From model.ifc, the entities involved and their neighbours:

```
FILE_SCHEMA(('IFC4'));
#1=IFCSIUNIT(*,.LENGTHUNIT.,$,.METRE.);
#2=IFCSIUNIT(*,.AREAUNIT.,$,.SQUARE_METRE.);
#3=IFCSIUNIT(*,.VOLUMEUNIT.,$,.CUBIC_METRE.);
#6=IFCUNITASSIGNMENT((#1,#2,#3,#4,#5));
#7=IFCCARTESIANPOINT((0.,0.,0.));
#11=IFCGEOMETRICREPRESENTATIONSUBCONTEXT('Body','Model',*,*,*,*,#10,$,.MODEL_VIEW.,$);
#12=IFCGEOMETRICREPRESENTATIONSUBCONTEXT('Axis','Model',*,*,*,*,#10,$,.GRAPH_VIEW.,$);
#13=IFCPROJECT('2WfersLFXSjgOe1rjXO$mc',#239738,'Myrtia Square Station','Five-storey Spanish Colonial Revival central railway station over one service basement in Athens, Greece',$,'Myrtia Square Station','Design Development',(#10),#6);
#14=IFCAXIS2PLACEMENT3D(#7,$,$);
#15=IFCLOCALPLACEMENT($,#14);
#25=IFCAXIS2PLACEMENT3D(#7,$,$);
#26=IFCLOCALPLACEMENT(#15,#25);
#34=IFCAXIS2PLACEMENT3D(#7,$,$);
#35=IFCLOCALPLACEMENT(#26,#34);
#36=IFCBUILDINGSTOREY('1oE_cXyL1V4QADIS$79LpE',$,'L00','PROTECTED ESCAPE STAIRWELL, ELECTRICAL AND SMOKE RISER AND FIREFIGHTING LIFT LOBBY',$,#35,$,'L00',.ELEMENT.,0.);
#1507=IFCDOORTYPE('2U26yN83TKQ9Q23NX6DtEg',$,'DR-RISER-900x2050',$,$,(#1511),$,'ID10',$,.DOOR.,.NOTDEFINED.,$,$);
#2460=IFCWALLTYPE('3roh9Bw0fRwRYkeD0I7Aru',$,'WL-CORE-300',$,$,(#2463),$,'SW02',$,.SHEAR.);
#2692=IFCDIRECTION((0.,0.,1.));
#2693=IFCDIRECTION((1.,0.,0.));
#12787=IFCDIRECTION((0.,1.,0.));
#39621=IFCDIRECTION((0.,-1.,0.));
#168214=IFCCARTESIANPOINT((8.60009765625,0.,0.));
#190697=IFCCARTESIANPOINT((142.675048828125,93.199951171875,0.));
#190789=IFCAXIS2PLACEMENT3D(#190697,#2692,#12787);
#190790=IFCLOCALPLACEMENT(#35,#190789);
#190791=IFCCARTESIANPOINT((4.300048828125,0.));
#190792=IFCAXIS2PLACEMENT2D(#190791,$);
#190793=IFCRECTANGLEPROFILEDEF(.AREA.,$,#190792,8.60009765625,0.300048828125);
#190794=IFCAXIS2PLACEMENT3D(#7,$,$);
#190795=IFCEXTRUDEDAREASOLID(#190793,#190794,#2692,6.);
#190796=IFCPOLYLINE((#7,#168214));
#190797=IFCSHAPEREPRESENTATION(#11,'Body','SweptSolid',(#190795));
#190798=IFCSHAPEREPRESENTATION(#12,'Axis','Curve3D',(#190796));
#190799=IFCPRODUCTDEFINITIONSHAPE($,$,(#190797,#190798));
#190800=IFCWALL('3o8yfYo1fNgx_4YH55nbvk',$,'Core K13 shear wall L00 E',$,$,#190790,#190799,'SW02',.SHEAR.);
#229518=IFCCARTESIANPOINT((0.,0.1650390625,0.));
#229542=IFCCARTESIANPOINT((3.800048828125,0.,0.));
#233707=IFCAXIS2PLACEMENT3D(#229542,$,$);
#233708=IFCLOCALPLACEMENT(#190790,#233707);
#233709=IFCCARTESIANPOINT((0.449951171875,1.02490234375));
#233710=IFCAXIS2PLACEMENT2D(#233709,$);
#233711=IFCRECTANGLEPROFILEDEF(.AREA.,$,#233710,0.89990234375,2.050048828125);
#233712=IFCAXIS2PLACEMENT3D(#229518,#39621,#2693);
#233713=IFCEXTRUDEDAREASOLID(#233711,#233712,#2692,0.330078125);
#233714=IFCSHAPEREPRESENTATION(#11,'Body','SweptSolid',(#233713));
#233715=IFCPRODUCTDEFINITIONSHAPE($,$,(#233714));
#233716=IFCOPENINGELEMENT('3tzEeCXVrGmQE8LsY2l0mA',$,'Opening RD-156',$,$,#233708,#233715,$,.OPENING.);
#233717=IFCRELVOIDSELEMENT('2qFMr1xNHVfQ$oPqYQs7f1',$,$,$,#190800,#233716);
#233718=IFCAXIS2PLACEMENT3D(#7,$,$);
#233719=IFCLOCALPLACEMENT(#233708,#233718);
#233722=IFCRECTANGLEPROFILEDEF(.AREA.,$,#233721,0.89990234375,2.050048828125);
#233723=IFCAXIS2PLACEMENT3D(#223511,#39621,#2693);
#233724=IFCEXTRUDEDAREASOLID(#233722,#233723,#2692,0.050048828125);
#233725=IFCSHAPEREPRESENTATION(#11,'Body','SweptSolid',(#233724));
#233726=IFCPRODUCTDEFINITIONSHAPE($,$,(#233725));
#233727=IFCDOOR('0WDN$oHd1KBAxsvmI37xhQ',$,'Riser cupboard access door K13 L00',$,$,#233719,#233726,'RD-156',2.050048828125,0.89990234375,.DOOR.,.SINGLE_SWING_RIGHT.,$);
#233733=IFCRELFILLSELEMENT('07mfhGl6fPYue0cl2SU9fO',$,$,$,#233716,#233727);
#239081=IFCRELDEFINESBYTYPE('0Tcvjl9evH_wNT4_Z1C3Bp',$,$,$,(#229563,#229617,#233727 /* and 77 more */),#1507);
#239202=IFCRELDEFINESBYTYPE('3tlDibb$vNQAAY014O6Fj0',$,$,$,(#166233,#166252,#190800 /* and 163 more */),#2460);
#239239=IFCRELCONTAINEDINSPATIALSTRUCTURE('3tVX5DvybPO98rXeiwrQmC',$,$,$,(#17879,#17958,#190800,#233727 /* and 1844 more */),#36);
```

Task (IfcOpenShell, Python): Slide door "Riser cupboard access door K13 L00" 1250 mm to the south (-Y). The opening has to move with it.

```python
import ifcopenshell
import ifcopenshell.api.geometry
import ifcopenshell.util.placement

model = ifcopenshell.open("model.ifc")

door = model.by_guid("0WDN$oHd1KBAxsvmI37xhQ")
opening = door.FillsVoids[0].RelatingOpeningElement
wall = opening.VoidsElements[0].RelatingBuildingElement

wall_matrix = ifcopenshell.util.placement.get_local_placement(wall.ObjectPlacement)
shift = wall_matrix[:3, 0] * -1.25
before = ifcopenshell.util.placement.get_local_placement(door.ObjectPlacement)[:3, 3].copy()

# The door is placed relative to its opening, so it follows when the opening moves.
matrix = ifcopenshell.util.placement.get_local_placement(opening.ObjectPlacement)
matrix[:3, 3] += shift
ifcopenshell.api.geometry.edit_object_placement(
    model, product=opening, matrix=matrix, is_si=False, should_transform_children=True
)

after = ifcopenshell.util.placement.get_local_placement(door.ObjectPlacement)[:3, 3]
print("door moved by", (after - before).round(3) + 0.0)

model.write("model_edited.ifc")
```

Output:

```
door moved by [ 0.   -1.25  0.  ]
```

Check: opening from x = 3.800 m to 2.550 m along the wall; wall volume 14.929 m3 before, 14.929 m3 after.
